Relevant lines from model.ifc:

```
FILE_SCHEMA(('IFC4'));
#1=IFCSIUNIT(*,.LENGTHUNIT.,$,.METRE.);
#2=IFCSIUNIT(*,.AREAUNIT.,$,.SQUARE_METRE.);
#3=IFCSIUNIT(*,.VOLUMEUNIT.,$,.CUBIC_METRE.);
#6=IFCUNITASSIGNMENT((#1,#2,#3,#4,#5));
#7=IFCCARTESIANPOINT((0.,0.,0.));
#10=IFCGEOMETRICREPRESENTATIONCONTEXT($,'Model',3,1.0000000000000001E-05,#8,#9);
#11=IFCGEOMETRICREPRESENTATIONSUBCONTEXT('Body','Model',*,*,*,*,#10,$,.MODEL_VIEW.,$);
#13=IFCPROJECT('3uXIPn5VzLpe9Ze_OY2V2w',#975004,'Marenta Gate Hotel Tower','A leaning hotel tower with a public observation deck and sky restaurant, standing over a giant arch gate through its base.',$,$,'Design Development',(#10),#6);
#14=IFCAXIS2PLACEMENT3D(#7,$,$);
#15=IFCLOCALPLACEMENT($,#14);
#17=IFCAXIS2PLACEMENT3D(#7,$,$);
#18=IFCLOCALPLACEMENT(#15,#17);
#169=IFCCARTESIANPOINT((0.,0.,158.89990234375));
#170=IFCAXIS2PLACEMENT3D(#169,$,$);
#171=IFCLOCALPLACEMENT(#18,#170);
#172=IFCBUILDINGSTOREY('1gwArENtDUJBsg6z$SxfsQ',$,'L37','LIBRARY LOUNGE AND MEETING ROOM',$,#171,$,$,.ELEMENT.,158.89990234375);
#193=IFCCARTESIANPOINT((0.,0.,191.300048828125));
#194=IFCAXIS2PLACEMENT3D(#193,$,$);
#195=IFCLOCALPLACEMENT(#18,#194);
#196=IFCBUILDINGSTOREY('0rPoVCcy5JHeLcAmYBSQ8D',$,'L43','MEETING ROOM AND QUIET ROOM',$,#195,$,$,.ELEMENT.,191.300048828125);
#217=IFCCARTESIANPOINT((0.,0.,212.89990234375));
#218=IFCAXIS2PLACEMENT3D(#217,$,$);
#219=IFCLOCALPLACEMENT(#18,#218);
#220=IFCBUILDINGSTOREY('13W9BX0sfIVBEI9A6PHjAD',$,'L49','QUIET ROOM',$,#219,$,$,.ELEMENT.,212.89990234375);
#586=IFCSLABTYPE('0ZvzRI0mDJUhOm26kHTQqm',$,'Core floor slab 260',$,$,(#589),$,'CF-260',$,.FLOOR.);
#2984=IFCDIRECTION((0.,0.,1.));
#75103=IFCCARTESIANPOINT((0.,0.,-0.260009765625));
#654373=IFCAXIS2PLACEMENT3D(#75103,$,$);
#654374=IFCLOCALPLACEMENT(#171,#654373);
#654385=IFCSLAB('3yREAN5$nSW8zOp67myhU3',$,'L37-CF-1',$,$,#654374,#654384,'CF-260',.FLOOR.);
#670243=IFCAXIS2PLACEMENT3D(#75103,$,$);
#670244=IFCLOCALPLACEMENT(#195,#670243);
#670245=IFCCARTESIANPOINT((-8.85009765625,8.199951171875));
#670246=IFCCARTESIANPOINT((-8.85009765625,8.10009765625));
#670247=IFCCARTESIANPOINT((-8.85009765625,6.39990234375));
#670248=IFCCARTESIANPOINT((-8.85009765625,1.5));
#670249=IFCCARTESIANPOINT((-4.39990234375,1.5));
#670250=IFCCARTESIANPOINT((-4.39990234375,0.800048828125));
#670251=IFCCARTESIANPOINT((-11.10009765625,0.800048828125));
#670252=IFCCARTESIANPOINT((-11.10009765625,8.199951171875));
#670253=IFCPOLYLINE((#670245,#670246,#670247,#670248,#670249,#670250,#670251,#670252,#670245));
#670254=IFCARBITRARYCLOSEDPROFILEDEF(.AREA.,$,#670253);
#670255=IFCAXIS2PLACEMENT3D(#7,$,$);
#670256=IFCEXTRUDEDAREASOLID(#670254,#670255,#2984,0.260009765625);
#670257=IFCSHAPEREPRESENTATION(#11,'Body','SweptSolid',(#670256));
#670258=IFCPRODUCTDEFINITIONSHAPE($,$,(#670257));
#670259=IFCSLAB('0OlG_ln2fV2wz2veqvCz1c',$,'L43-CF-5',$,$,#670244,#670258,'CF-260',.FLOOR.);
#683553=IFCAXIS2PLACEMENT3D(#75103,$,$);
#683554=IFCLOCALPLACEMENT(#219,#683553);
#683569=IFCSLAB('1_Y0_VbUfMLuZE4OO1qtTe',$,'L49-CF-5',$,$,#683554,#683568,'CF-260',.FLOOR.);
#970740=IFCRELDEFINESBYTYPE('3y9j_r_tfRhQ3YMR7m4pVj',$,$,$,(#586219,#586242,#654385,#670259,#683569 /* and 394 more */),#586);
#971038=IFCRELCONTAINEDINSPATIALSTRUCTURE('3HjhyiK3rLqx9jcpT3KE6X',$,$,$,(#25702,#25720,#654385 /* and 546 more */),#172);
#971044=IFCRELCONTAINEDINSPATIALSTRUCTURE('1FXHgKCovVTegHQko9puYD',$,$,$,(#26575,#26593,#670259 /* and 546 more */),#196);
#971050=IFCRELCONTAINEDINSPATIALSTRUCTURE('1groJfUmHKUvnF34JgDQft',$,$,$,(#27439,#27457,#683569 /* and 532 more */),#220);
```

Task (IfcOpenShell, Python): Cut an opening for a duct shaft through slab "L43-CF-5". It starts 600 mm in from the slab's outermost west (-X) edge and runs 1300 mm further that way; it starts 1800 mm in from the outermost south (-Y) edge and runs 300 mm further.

```python
import numpy as np
import ifcopenshell
import ifcopenshell.api.feature
import ifcopenshell.api.geometry
import ifcopenshell.api.root
import ifcopenshell.geom
import ifcopenshell.util.placement
import ifcopenshell.util.representation
import ifcopenshell.util.shape
import ifcopenshell.util.unit

model = ifcopenshell.open("model.ifc")
unit_scale = ifcopenshell.util.unit.calculate_unit_scale(model)
settings = ifcopenshell.geom.settings()


def volume(element):
    """Net volume in cubic metres, openings subtracted."""
    shape = ifcopenshell.geom.create_shape(settings, element)
    return ifcopenshell.util.shape.get_volume(shape.geometry)


slab = model.by_id(670259)
before = volume(slab)

# Extent in the slab's own axes, in metres. The edges named are its -X and -Y sides.
slab_shape = ifcopenshell.geom.create_shape(settings, slab)
vertices = ifcopenshell.util.shape.get_vertices(slab_shape.geometry)
x_min, y_min, bottom = vertices.min(axis=0)
top = vertices[:, 2].max()

opening = ifcopenshell.api.root.create_entity(model, ifc_class="IfcOpeningElement", name="Duct shaft opening", predefined_type="OPENING")
context = ifcopenshell.util.representation.get_context(model, "Model", "Body", "MODEL_VIEW")
width, depth = 1.3, 0.3
outline = [(0.0, 0.0), (width, 0.0), (width, depth), (0.0, depth), (0.0, 0.0)]
# Overshoot both faces by 50 mm so the cut is clean.
shape = ifcopenshell.api.geometry.add_slab_representation(
    model, context=context, depth=top - bottom + 0.1, polyline=outline
)
ifcopenshell.api.geometry.assign_representation(model, product=opening, representation=shape)

matrix = ifcopenshell.util.placement.get_local_placement(slab.ObjectPlacement)
matrix[:, 3] = matrix @ np.append(np.array([x_min + 0.6, y_min + 1.8, bottom - 0.05]) / unit_scale, 1.0)
ifcopenshell.api.geometry.edit_object_placement(model, product=opening, matrix=matrix, is_si=False)
ifcopenshell.api.feature.add_feature(model, feature=opening, element=slab)

after = volume(slab)

print(f"slab volume {before:.3f} -> {after:.3f} m3")

model.write("model_rev.ifc")
```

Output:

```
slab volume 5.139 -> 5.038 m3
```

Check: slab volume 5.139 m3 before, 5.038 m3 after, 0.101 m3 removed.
